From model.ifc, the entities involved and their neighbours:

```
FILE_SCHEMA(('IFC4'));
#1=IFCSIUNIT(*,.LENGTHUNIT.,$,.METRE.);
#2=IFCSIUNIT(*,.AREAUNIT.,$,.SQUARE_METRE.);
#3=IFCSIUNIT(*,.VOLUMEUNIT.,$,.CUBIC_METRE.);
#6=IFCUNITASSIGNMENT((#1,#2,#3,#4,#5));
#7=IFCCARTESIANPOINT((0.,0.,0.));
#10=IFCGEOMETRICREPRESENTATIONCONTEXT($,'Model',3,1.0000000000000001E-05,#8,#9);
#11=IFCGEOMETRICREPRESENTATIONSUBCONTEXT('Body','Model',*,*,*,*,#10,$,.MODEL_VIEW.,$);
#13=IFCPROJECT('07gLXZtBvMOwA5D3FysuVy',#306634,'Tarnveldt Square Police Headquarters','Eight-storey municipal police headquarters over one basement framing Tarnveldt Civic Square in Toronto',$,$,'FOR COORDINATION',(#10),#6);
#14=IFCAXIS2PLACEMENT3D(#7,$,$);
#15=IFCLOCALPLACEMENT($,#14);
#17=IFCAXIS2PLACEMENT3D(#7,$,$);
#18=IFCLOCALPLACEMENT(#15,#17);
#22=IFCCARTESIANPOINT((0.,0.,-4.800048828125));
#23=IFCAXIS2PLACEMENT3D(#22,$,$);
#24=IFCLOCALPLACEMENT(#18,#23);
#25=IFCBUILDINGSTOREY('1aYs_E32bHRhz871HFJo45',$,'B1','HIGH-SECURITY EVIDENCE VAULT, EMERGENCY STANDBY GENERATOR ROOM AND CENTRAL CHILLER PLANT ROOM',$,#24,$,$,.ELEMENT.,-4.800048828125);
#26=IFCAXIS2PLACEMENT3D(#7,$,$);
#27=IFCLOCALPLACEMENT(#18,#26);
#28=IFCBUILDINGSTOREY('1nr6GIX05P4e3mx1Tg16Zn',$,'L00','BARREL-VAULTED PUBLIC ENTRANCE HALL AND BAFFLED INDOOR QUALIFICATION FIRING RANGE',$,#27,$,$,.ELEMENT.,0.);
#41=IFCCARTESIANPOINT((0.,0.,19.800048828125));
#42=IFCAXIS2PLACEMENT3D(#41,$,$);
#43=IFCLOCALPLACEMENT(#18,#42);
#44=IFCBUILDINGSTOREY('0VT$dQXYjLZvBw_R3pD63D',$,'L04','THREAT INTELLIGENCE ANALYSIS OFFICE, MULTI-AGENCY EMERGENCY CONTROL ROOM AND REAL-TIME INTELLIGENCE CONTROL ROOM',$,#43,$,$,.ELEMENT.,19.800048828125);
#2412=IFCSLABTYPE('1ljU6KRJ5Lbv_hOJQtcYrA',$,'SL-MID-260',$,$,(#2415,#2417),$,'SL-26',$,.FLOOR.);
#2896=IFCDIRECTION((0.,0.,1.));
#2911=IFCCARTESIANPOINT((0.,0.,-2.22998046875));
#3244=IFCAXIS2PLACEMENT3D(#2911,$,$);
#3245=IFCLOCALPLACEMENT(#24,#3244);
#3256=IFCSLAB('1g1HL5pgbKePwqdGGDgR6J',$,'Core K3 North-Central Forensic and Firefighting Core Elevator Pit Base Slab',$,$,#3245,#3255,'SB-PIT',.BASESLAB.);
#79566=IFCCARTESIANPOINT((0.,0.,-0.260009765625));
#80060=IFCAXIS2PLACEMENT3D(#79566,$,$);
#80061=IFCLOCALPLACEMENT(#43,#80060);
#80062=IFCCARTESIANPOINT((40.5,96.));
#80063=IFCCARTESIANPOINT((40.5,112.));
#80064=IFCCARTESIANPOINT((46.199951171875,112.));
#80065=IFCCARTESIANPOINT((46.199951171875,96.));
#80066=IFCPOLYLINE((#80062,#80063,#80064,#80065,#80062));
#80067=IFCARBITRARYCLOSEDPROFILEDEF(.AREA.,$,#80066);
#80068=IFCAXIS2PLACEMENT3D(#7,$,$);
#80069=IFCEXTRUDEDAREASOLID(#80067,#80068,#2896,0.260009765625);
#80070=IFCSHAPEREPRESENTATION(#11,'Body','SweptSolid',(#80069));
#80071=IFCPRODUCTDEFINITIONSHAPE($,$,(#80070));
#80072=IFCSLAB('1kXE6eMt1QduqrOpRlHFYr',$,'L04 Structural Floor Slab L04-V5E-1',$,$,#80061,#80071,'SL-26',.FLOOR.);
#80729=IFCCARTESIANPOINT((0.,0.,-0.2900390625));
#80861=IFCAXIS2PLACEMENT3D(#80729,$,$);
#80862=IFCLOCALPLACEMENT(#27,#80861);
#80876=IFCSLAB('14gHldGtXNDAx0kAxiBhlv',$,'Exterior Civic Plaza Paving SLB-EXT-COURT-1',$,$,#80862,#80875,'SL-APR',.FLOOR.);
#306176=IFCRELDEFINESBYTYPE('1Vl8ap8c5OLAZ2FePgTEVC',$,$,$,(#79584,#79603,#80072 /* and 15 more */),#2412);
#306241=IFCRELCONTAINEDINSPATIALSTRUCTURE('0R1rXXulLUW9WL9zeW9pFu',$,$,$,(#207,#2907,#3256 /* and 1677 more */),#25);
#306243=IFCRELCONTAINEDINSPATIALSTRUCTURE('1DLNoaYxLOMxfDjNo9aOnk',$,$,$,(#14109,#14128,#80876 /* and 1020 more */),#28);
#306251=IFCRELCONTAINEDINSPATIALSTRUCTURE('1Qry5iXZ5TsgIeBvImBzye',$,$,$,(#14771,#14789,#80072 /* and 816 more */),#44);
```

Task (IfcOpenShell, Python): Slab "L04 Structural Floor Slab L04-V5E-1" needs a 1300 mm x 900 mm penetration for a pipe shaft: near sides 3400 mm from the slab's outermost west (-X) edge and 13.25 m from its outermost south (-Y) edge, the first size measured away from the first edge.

```python
import numpy as np
import ifcopenshell
import ifcopenshell.api.feature
import ifcopenshell.api.geometry
import ifcopenshell.api.root
import ifcopenshell.geom
import ifcopenshell.util.placement
import ifcopenshell.util.representation
import ifcopenshell.util.shape
import ifcopenshell.util.unit

model = ifcopenshell.open("model.ifc")
unit_scale = ifcopenshell.util.unit.calculate_unit_scale(model)
settings = ifcopenshell.geom.settings()


def volume(element):
    """Net volume in cubic metres, openings subtracted."""
    shape = ifcopenshell.geom.create_shape(settings, element)
    return ifcopenshell.util.shape.get_volume(shape.geometry)


slab = model.by_guid("1kXE6eMt1QduqrOpRlHFYr")
before = volume(slab)

# Extent in the slab's own axes, in metres. The edges named are its -X and -Y sides.
slab_shape = ifcopenshell.geom.create_shape(settings, slab)
vertices = ifcopenshell.util.shape.get_vertices(slab_shape.geometry)
x_min, y_min, bottom = vertices.min(axis=0)
top = vertices[:, 2].max()

opening = ifcopenshell.api.root.create_entity(model, ifc_class="IfcOpeningElement", name="Pipe shaft opening", predefined_type="OPENING")
context = ifcopenshell.util.representation.get_context(model, "Model", "Body", "MODEL_VIEW")
width, depth = 1.3, 0.9
outline = [(0.0, 0.0), (width, 0.0), (width, depth), (0.0, depth), (0.0, 0.0)]
# Overshoot both faces by 50 mm so the cut is clean.
shape = ifcopenshell.api.geometry.add_slab_representation(
    model, context=context, depth=top - bottom + 0.1, polyline=outline
)
ifcopenshell.api.geometry.assign_representation(model, product=opening, representation=shape)

matrix = ifcopenshell.util.placement.get_local_placement(slab.ObjectPlacement)
matrix[:, 3] = matrix @ np.append(np.array([x_min + 3.4, y_min + 13.25, bottom - 0.05]) / unit_scale, 1.0)
ifcopenshell.api.geometry.edit_object_placement(model, product=opening, matrix=matrix, is_si=False)
ifcopenshell.api.feature.add_feature(model, feature=opening, element=slab)

after = volume(slab)

print(f"slab volume {before:.3f} -> {after:.3f} m3")

model.write("model_v2.ifc")
```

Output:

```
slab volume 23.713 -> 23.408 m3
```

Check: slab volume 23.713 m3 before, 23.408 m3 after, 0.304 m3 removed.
